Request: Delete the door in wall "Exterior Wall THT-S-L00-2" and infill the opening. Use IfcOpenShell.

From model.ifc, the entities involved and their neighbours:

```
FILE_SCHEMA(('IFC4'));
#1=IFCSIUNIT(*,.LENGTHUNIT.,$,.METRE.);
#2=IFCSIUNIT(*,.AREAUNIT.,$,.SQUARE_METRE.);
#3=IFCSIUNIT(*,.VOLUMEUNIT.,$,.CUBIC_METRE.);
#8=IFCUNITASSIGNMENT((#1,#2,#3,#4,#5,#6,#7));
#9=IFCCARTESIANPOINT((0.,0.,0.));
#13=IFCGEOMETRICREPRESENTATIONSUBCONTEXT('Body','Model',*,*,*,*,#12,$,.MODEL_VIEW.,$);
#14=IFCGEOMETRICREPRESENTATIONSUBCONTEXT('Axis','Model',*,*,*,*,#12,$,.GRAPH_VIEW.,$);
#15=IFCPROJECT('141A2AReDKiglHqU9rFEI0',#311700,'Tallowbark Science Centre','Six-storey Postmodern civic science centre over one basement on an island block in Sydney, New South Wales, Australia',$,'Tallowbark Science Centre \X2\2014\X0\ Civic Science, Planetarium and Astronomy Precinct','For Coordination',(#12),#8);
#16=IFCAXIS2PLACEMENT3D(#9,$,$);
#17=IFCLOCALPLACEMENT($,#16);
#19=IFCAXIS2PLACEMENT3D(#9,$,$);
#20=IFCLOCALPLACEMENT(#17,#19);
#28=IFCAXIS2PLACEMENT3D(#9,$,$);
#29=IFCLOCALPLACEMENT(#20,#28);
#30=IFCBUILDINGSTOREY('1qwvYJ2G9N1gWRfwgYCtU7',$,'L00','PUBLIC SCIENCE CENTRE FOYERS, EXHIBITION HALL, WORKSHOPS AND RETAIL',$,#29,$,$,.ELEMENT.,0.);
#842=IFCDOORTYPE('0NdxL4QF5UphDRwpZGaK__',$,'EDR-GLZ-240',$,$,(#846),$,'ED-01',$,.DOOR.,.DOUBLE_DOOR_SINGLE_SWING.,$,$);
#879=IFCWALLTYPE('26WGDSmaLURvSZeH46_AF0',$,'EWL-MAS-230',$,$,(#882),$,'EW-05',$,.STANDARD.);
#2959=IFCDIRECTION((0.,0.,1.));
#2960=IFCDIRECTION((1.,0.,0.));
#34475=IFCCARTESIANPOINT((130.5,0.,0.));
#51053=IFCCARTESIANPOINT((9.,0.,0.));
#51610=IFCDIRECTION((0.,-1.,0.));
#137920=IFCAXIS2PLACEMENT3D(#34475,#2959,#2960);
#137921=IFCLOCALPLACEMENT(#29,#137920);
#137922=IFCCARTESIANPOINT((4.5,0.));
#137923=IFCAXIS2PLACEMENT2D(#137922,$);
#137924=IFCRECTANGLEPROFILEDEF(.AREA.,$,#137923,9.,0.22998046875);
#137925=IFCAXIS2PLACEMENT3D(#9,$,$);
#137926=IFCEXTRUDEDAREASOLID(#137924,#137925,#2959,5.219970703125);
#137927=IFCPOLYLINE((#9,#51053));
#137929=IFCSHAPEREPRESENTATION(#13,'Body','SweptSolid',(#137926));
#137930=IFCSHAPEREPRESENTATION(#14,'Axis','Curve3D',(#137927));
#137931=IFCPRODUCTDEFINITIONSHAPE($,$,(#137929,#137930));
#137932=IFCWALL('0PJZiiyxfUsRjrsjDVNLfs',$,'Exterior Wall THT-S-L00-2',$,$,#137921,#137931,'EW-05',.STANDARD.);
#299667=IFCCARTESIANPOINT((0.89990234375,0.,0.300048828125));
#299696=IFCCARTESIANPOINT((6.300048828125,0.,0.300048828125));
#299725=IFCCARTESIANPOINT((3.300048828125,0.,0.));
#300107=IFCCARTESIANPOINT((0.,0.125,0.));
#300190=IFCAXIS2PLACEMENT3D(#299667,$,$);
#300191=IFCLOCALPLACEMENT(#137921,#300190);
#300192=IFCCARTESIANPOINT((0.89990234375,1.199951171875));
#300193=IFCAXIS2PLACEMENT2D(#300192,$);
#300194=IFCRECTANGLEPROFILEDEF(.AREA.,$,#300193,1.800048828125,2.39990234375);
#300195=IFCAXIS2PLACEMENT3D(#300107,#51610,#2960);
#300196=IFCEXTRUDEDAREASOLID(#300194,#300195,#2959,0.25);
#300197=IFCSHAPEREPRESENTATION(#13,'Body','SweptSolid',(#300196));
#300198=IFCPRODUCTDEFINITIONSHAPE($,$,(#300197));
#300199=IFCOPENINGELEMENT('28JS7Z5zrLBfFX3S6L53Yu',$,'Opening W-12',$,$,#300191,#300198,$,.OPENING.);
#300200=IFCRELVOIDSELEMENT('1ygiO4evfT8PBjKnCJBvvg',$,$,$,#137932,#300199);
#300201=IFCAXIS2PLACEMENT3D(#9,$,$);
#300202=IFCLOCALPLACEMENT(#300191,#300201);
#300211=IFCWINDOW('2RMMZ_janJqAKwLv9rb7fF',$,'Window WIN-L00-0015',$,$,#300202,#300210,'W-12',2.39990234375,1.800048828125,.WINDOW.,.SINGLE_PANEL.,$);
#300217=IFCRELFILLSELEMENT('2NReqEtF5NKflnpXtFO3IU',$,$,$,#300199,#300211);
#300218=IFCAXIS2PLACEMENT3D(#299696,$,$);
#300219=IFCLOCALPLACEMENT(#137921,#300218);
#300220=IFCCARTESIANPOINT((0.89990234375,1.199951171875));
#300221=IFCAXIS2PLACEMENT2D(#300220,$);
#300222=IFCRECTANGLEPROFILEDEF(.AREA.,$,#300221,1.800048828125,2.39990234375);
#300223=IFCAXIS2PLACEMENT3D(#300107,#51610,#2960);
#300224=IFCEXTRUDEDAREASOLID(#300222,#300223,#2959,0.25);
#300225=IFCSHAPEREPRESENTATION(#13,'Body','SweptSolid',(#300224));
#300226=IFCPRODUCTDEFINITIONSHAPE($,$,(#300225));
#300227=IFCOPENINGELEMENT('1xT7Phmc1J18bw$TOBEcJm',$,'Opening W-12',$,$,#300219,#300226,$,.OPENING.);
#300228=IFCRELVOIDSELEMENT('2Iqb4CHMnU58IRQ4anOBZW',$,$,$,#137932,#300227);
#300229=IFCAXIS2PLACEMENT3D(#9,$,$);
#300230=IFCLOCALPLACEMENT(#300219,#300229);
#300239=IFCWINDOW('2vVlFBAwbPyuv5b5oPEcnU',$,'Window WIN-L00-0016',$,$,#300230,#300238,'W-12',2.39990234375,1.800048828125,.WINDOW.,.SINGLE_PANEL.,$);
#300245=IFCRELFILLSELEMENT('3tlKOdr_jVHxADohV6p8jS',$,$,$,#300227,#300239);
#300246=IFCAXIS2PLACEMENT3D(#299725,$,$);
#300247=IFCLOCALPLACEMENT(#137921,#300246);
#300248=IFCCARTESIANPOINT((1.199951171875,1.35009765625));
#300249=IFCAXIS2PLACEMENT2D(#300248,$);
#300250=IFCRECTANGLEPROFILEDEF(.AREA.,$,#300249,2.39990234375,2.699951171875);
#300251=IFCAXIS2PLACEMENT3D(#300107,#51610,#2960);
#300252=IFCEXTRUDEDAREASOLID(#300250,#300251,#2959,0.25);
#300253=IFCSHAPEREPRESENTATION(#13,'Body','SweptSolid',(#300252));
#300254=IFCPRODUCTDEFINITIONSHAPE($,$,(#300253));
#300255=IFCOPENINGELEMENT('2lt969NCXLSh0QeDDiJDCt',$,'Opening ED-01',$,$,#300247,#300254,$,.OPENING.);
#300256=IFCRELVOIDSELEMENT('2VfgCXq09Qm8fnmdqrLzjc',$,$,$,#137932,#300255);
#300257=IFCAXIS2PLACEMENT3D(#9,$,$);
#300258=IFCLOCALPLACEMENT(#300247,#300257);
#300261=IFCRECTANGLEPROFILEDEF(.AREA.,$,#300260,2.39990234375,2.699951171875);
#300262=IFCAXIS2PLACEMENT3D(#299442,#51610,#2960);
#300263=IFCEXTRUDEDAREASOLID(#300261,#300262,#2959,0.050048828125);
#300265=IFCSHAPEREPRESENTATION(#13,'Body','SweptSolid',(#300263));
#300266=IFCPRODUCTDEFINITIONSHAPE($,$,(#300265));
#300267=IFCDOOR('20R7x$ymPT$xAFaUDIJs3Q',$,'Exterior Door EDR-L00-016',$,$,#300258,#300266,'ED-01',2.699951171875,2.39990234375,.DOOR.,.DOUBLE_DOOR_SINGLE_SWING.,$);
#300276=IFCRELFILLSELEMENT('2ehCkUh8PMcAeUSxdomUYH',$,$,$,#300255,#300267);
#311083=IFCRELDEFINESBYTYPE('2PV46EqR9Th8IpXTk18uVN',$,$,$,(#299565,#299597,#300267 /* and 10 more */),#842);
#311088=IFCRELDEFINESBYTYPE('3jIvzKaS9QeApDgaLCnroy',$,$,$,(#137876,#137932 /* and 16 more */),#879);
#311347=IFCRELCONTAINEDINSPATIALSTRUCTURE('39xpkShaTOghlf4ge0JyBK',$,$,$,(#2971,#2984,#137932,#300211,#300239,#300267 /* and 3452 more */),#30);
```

```python
import ifcopenshell
import ifcopenshell.api.feature
import ifcopenshell.api.root
import ifcopenshell.geom
import ifcopenshell.util.shape

model = ifcopenshell.open("model.ifc")
settings = ifcopenshell.geom.settings()


def volume(element):
    """Net volume in cubic metres, openings subtracted."""
    shape = ifcopenshell.geom.create_shape(settings, element)
    return ifcopenshell.util.shape.get_volume(shape.geometry)


door = model.by_guid("20R7x$ymPT$xAFaUDIJs3Q")
opening = door.FillsVoids[0].RelatingOpeningElement
wall = opening.VoidsElements[0].RelatingBuildingElement
before = volume(wall)

ifcopenshell.api.root.remove_product(model, product=door)
ifcopenshell.api.feature.remove_feature(model, feature=opening)

after = volume(wall)

print(f"wall volume {before:.3f} -> {after:.3f} m3")

model.write("model_rev.ifc")
```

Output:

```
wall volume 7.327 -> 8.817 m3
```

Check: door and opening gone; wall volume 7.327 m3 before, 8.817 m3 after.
